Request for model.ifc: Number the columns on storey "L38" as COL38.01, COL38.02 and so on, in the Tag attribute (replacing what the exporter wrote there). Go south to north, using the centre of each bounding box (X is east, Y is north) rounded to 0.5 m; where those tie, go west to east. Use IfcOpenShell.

First a look at what the model holds.

```python
import ifcopenshell
import ifcopenshell.util.element
import ifcopenshell.util.placement

model = ifcopenshell.open("model.ifc")
print(model.schema)
storey = next(s for s in model.by_type("IfcBuildingStorey") if s.Name == "L38")
columns = [e for e in ifcopenshell.util.element.get_decomposition(storey) if e.is_a("IfcColumn")]
for e in sorted(columns, key=lambda e: e.id()):
    origin = ifcopenshell.util.placement.get_local_placement(e.ObjectPlacement)[:3, 3]
    print(e.id(), e.Tag, e.Name, origin.round(2) + 0.0, sep=" | ")
```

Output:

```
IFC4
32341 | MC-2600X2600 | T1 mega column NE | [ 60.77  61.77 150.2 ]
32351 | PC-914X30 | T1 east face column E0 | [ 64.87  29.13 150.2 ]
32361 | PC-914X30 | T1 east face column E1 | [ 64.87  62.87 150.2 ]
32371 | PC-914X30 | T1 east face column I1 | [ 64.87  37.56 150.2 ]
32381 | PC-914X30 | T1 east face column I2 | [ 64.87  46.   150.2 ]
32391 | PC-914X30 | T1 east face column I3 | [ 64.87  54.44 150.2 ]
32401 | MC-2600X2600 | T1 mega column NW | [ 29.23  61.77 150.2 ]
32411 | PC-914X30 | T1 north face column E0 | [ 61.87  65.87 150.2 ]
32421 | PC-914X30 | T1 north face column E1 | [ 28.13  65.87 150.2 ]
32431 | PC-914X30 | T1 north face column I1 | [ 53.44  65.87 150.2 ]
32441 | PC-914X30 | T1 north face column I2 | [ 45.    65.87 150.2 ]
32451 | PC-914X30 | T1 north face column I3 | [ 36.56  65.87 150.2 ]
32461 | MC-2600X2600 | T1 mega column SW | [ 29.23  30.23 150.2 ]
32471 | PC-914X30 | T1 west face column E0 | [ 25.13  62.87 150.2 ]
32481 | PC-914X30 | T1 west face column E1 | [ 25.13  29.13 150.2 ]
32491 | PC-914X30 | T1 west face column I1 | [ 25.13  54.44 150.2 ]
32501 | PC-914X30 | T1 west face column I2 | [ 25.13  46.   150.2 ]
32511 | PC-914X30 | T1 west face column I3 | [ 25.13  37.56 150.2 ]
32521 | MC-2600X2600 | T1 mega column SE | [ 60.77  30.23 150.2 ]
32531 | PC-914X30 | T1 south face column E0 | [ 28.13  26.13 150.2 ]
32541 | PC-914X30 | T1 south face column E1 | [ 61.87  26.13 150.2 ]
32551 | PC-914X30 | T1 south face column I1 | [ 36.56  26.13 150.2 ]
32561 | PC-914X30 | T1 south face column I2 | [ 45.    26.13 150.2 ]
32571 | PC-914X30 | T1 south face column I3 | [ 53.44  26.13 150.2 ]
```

```python
import ifcopenshell
import ifcopenshell.geom
import ifcopenshell.util.element
import ifcopenshell.util.shape

model = ifcopenshell.open("model.ifc")
settings = ifcopenshell.geom.settings()
settings.set("use-world-coords", True)


def centre(element):
    shape = ifcopenshell.geom.create_shape(settings, element)
    return ifcopenshell.util.shape.get_bbox_centroid(shape.geometry)


storey = next(s for s in model.by_type("IfcBuildingStorey") if s.Name == "L38")
columns = [e for e in ifcopenshell.util.element.get_decomposition(storey) if e.is_a("IfcColumn")]

# Insertion points can sit at a corner or the storey origin, so sort by the geometry (in metres).
centres = {e: centre(e) for e in columns}
columns.sort(key=lambda e: (round(centres[e][1] / 0.5), centres[e][0]))

for i, e in enumerate(columns, start=1):
    number = f"COL38.{i:02d}"
    e.Tag = number
    print(e.id(), number)

model.write("model_v2.ifc")
```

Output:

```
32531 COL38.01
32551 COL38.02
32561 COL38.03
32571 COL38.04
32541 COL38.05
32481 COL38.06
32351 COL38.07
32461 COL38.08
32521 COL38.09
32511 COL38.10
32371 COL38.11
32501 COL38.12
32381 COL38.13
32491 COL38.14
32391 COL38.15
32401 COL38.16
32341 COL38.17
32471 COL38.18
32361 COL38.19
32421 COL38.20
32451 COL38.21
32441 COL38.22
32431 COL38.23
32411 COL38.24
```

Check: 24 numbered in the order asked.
